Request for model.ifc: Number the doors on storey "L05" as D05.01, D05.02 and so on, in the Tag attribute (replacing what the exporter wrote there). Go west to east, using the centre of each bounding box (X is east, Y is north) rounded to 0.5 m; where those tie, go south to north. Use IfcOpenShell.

First a look at what the model holds.

```python
import ifcopenshell
import ifcopenshell.util.element
import ifcopenshell.util.placement

model = ifcopenshell.open("model.ifc")
print(model.schema)
storey = next(s for s in model.by_type("IfcBuildingStorey") if s.Name == "L05")
doors = [e for e in ifcopenshell.util.element.get_decomposition(storey) if e.is_a("IfcDoor")]
for e in sorted(doors, key=lambda e: e.id()):
    origin = ifcopenshell.util.placement.get_local_placement(e.ObjectPlacement)[:3, 3]
    print(e.id(), e.Tag, e.Name, origin.round(2) + 0.0, sep=" | ")
```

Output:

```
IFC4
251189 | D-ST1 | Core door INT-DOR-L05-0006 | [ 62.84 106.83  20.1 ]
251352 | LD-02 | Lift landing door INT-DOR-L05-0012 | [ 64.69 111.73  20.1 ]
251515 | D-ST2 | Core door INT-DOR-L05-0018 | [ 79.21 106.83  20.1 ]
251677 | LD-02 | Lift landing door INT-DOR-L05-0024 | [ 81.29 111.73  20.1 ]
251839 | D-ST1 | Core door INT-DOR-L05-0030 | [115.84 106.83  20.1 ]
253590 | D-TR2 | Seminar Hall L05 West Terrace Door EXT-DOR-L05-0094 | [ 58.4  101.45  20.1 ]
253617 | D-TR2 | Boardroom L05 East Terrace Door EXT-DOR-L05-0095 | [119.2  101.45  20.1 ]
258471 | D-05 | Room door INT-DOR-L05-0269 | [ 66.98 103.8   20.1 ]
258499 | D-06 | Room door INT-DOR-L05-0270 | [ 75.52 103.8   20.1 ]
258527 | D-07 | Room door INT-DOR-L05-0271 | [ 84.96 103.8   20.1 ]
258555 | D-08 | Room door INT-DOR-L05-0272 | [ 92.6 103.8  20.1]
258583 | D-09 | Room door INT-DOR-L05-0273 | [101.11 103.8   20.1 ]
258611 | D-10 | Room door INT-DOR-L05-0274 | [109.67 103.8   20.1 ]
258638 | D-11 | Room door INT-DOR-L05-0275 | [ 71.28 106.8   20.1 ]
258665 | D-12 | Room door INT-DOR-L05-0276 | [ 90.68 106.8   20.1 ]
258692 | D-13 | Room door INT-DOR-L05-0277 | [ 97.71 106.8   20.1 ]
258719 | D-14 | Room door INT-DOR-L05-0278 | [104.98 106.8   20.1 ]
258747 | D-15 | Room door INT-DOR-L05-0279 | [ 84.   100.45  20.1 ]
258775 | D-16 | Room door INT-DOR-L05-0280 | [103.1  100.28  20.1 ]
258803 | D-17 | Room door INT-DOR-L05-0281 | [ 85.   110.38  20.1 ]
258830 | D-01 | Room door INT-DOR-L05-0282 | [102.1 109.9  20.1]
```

```python
import ifcopenshell
import ifcopenshell.geom
import ifcopenshell.util.element
import ifcopenshell.util.shape

model = ifcopenshell.open("model.ifc")
settings = ifcopenshell.geom.settings()
settings.set("use-world-coords", True)


def centre(element):
    shape = ifcopenshell.geom.create_shape(settings, element)
    return ifcopenshell.util.shape.get_bbox_centroid(shape.geometry)


storey = next(s for s in model.by_type("IfcBuildingStorey") if s.Name == "L05")
doors = [e for e in ifcopenshell.util.element.get_decomposition(storey) if e.is_a("IfcDoor")]

# Insertion points can sit at a corner or the storey origin, so sort by the geometry (in metres).
centres = {e: centre(e) for e in doors}
doors.sort(key=lambda e: (round(centres[e][0] / 0.5), centres[e][1]))

for i, e in enumerate(doors, start=1):
    number = f"D05.{i:02d}"
    e.Tag = number
    print(e.id(), number)

model.write("model_updated.ifc")
```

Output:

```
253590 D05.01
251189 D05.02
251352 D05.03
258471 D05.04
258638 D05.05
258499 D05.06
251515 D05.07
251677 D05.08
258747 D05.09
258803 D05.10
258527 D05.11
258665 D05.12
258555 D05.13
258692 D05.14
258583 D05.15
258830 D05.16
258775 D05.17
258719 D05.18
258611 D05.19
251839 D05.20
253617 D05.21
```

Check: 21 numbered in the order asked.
